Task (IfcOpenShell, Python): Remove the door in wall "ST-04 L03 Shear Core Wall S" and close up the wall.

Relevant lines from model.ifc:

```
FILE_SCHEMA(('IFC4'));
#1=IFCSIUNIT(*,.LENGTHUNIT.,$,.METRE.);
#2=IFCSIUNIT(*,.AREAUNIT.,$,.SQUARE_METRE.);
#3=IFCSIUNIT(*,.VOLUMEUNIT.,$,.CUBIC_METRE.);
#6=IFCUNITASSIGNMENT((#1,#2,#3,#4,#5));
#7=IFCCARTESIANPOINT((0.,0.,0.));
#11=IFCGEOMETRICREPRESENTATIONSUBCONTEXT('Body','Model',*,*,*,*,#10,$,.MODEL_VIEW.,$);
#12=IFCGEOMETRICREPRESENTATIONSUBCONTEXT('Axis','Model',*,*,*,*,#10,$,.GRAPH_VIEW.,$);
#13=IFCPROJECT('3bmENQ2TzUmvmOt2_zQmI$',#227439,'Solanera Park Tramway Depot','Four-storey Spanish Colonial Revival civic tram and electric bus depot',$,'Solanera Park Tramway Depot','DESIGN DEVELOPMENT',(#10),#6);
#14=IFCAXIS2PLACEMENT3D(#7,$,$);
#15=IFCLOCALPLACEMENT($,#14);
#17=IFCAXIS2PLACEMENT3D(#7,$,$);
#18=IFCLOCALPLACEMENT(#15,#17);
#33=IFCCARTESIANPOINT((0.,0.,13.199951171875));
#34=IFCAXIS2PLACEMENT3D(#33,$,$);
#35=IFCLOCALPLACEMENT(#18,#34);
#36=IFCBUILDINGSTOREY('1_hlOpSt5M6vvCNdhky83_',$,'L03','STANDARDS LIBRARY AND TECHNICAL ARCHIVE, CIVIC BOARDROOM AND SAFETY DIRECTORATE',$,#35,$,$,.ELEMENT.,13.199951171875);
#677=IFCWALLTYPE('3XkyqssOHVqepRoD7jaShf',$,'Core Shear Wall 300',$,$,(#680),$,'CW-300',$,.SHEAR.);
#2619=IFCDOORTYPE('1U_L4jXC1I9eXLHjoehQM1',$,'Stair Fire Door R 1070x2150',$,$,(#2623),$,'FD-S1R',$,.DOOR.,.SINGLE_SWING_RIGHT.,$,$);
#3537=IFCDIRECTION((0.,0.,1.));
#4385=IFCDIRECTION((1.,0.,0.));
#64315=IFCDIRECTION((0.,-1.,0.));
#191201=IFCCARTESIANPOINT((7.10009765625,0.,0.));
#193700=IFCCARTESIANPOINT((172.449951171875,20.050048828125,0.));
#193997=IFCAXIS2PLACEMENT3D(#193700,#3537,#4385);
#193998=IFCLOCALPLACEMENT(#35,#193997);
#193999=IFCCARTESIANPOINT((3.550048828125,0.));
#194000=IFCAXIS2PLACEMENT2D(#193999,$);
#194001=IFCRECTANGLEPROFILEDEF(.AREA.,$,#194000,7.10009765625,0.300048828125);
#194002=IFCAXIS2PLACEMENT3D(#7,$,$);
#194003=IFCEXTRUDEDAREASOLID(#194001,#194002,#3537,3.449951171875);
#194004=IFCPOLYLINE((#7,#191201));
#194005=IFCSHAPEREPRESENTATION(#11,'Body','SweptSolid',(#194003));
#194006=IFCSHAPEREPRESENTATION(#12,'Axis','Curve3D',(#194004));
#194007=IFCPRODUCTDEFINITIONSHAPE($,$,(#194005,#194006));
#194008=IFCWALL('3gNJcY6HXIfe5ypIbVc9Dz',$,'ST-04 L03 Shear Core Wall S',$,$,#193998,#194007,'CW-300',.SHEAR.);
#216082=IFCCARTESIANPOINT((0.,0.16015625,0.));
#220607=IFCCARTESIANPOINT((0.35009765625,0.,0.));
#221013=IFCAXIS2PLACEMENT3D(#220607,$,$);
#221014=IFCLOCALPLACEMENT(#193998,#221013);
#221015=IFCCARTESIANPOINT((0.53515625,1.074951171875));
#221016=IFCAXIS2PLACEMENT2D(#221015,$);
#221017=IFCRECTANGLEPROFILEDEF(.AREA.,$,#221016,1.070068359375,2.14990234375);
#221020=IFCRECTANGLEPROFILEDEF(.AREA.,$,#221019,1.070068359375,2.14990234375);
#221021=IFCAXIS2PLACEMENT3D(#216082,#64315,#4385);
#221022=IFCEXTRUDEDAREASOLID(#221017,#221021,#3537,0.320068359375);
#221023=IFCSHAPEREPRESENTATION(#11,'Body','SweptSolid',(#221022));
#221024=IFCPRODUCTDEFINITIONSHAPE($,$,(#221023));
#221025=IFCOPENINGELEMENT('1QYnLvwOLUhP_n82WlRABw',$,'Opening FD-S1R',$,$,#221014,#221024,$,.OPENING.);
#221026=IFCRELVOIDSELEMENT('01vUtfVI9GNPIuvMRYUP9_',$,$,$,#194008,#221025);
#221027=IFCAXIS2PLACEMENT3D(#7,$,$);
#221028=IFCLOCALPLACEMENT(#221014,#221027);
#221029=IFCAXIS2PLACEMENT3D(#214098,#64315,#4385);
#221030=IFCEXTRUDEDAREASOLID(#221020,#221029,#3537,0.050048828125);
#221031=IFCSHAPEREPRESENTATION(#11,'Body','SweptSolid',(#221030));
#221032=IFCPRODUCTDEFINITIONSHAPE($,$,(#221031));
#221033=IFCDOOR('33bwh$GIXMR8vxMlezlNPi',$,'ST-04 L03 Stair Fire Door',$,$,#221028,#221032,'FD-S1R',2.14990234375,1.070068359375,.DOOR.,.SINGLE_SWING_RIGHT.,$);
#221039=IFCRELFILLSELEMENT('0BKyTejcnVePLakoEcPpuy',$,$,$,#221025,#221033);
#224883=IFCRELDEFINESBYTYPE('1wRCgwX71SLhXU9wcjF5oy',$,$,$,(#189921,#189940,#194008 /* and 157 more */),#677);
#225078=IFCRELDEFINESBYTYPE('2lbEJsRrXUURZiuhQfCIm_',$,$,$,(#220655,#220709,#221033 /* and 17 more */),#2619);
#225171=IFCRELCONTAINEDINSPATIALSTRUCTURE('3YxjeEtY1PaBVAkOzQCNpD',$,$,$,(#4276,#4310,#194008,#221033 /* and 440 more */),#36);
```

```python
import ifcopenshell
import ifcopenshell.api.feature
import ifcopenshell.api.root
import ifcopenshell.geom
import ifcopenshell.util.shape

model = ifcopenshell.open("model.ifc")
settings = ifcopenshell.geom.settings()


def volume(element):
    """Net volume in cubic metres, openings subtracted."""
    shape = ifcopenshell.geom.create_shape(settings, element)
    return ifcopenshell.util.shape.get_volume(shape.geometry)


door = model.by_id(221033)
opening = door.FillsVoids[0].RelatingOpeningElement
wall = opening.VoidsElements[0].RelatingBuildingElement
before = volume(wall)

ifcopenshell.api.root.remove_product(model, product=door)
ifcopenshell.api.feature.remove_feature(model, feature=opening)

after = volume(wall)

print(f"wall volume {before:.3f} -> {after:.3f} m3")

model.write("model_v2.ifc")
```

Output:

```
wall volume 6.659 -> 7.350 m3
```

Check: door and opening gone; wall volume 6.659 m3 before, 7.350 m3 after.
